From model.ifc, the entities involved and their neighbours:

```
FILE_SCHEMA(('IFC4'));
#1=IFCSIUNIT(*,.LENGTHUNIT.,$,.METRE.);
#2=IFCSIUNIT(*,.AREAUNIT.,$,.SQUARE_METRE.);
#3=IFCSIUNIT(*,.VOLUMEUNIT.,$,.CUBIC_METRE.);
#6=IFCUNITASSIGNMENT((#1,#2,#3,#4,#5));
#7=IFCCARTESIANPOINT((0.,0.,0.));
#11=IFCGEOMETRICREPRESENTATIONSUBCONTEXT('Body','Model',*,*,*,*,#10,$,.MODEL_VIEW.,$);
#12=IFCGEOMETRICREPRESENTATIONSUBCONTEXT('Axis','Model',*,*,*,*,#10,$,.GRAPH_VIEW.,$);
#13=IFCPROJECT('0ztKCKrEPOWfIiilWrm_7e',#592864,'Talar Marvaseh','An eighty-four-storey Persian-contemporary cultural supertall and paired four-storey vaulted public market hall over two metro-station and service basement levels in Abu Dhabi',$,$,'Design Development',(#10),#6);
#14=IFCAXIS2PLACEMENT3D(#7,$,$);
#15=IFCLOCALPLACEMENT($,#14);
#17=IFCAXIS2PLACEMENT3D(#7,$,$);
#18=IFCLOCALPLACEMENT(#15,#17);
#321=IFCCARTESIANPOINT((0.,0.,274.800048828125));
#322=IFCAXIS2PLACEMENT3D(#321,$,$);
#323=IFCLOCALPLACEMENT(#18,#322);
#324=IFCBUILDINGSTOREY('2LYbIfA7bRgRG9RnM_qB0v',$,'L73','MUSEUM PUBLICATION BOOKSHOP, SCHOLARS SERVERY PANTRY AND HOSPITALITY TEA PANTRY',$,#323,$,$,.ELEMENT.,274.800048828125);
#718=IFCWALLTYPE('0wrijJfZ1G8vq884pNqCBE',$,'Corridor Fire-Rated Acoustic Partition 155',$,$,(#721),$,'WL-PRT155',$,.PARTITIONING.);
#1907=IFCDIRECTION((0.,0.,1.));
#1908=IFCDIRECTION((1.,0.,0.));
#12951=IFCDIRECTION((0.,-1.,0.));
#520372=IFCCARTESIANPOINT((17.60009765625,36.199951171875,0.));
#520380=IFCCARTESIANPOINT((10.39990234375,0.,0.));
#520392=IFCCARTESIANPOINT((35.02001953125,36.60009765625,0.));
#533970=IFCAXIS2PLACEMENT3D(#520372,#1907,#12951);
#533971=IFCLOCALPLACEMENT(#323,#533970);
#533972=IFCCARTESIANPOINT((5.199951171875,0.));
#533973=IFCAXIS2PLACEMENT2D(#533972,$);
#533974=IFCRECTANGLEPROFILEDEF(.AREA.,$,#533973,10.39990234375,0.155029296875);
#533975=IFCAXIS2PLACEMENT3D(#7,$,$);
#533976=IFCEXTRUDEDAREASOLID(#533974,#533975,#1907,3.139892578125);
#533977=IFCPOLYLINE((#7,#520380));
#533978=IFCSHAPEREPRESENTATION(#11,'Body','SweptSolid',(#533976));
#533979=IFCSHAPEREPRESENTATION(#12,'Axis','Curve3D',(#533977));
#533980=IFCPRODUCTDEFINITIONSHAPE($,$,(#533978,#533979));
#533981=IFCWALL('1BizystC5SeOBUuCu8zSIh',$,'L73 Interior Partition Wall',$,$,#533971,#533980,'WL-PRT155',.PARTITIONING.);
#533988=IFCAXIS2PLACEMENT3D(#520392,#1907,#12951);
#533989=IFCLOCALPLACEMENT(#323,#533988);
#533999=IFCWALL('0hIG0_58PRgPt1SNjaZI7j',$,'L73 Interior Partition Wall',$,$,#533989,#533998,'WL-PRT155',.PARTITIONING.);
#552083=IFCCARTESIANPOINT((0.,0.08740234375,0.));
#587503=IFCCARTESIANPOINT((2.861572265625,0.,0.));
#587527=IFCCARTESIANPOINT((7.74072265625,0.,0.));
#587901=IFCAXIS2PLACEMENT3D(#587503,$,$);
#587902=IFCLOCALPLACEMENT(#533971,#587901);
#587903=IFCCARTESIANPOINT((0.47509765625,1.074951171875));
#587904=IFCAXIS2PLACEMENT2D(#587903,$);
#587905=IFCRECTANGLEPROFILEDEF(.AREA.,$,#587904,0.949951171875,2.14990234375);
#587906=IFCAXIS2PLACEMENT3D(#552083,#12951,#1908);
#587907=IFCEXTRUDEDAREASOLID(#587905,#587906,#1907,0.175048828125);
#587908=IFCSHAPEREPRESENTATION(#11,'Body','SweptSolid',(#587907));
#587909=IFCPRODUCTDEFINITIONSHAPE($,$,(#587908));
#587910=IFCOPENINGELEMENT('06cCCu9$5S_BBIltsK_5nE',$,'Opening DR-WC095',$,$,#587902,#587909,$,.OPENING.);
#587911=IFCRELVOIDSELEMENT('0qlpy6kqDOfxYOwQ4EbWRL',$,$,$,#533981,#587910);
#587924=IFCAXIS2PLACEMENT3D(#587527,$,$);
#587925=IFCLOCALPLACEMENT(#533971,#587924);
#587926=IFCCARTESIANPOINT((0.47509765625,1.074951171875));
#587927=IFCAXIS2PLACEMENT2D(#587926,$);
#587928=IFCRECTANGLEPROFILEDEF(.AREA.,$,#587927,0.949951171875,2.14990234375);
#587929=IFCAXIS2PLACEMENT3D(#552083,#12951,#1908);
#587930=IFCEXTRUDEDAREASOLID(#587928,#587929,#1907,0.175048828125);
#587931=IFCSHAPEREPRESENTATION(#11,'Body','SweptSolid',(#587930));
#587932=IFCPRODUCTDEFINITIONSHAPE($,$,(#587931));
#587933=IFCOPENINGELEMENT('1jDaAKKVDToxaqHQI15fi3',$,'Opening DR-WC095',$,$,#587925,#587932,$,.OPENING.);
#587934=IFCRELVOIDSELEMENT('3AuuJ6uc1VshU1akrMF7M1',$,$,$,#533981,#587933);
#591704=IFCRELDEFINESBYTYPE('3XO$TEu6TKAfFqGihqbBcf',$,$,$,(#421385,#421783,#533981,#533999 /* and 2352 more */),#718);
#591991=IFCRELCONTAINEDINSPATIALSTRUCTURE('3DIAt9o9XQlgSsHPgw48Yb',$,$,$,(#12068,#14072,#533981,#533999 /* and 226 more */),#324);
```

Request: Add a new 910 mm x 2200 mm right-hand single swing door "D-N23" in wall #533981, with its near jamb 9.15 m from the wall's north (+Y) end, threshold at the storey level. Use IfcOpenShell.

```python
import numpy as np
import ifcopenshell
import ifcopenshell.api.feature
import ifcopenshell.api.geometry
import ifcopenshell.api.root
import ifcopenshell.api.spatial
import ifcopenshell.geom
import ifcopenshell.util.element
import ifcopenshell.util.placement
import ifcopenshell.util.representation
import ifcopenshell.util.shape
import ifcopenshell.util.unit

model = ifcopenshell.open("model.ifc")
unit_scale = ifcopenshell.util.unit.calculate_unit_scale(model)
settings = ifcopenshell.geom.settings()


def volume(element):
    """Net volume in cubic metres, openings subtracted."""
    shape = ifcopenshell.geom.create_shape(settings, element)
    return ifcopenshell.util.shape.get_volume(shape.geometry)


wall = model.by_guid("1BizystC5SeOBUuCu8zSIh")
storey = ifcopenshell.util.element.get_container(wall, ifc_class="IfcBuildingStorey")
context = ifcopenshell.util.representation.get_context(model, "Model", "Body", "MODEL_VIEW")
before = volume(wall)

width, height, from_end, sill = 0.91, 2.2, 9.15, 0.0  # metres

# The wall runs along its own X axis, and the end named is its -X end.
wall_shape = ifcopenshell.geom.create_shape(settings, wall)
x, y, z = ifcopenshell.util.shape.get_vertices(wall_shape.geometry).T
start = x.min() + from_end
face, thickness = float(y.min()), float(y.max() - y.min())
wall_matrix = ifcopenshell.util.placement.get_local_placement(wall.ObjectPlacement)
level = ifcopenshell.util.placement.get_local_placement(storey.ObjectPlacement)[2, 3]


def in_wall(x, y):
    """Placement at x, y metres in the wall's axes, at sill height."""
    matrix = wall_matrix.copy()
    matrix[:, 3] = wall_matrix @ np.array([x / unit_scale, y / unit_scale, 0.0, 1.0])
    matrix[2, 3] = level + sill / unit_scale
    return matrix


# Opening: a box that overshoots both wall faces by 50 mm.
opening = ifcopenshell.api.root.create_entity(model, ifc_class="IfcOpeningElement", predefined_type="OPENING")
box = ifcopenshell.api.geometry.add_wall_representation(
    model, context=context, length=width, height=height, thickness=thickness + 0.1
)
ifcopenshell.api.geometry.assign_representation(model, product=opening, representation=box)
ifcopenshell.api.geometry.edit_object_placement(model, product=opening, matrix=in_wall(start, face - 0.05), is_si=False)
ifcopenshell.api.feature.add_feature(model, feature=opening, element=wall)

door = ifcopenshell.api.root.create_entity(model, ifc_class="IfcDoor", name="D-N23", predefined_type="DOOR")
door.OverallWidth, door.OverallHeight = width / unit_scale, height / unit_scale
door.OperationType = "SINGLE_SWING_RIGHT"
body = ifcopenshell.api.geometry.add_door_representation(
    model,
    context=context,
    overall_width=door.OverallWidth,
    overall_height=door.OverallHeight,
    operation_type="SINGLE_SWING_RIGHT",
    lining_properties={"LiningDepth": thickness / unit_scale, "ThresholdDepth": thickness / unit_scale},
)
ifcopenshell.api.geometry.assign_representation(model, product=door, representation=body)
ifcopenshell.api.spatial.assign_container(model, products=[door], relating_structure=storey)
ifcopenshell.api.feature.add_filling(model, opening=opening, element=door)

# The lining spans the wall, so the door starts at the wall face.
ifcopenshell.api.geometry.edit_object_placement(model, product=door, matrix=in_wall(start, face), is_si=False)

after = volume(wall)

print(f"wall volume {before:.3f} -> {after:.3f} m3")

model.write("model-out.ifc")
```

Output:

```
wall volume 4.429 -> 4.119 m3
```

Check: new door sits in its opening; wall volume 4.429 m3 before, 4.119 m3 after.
